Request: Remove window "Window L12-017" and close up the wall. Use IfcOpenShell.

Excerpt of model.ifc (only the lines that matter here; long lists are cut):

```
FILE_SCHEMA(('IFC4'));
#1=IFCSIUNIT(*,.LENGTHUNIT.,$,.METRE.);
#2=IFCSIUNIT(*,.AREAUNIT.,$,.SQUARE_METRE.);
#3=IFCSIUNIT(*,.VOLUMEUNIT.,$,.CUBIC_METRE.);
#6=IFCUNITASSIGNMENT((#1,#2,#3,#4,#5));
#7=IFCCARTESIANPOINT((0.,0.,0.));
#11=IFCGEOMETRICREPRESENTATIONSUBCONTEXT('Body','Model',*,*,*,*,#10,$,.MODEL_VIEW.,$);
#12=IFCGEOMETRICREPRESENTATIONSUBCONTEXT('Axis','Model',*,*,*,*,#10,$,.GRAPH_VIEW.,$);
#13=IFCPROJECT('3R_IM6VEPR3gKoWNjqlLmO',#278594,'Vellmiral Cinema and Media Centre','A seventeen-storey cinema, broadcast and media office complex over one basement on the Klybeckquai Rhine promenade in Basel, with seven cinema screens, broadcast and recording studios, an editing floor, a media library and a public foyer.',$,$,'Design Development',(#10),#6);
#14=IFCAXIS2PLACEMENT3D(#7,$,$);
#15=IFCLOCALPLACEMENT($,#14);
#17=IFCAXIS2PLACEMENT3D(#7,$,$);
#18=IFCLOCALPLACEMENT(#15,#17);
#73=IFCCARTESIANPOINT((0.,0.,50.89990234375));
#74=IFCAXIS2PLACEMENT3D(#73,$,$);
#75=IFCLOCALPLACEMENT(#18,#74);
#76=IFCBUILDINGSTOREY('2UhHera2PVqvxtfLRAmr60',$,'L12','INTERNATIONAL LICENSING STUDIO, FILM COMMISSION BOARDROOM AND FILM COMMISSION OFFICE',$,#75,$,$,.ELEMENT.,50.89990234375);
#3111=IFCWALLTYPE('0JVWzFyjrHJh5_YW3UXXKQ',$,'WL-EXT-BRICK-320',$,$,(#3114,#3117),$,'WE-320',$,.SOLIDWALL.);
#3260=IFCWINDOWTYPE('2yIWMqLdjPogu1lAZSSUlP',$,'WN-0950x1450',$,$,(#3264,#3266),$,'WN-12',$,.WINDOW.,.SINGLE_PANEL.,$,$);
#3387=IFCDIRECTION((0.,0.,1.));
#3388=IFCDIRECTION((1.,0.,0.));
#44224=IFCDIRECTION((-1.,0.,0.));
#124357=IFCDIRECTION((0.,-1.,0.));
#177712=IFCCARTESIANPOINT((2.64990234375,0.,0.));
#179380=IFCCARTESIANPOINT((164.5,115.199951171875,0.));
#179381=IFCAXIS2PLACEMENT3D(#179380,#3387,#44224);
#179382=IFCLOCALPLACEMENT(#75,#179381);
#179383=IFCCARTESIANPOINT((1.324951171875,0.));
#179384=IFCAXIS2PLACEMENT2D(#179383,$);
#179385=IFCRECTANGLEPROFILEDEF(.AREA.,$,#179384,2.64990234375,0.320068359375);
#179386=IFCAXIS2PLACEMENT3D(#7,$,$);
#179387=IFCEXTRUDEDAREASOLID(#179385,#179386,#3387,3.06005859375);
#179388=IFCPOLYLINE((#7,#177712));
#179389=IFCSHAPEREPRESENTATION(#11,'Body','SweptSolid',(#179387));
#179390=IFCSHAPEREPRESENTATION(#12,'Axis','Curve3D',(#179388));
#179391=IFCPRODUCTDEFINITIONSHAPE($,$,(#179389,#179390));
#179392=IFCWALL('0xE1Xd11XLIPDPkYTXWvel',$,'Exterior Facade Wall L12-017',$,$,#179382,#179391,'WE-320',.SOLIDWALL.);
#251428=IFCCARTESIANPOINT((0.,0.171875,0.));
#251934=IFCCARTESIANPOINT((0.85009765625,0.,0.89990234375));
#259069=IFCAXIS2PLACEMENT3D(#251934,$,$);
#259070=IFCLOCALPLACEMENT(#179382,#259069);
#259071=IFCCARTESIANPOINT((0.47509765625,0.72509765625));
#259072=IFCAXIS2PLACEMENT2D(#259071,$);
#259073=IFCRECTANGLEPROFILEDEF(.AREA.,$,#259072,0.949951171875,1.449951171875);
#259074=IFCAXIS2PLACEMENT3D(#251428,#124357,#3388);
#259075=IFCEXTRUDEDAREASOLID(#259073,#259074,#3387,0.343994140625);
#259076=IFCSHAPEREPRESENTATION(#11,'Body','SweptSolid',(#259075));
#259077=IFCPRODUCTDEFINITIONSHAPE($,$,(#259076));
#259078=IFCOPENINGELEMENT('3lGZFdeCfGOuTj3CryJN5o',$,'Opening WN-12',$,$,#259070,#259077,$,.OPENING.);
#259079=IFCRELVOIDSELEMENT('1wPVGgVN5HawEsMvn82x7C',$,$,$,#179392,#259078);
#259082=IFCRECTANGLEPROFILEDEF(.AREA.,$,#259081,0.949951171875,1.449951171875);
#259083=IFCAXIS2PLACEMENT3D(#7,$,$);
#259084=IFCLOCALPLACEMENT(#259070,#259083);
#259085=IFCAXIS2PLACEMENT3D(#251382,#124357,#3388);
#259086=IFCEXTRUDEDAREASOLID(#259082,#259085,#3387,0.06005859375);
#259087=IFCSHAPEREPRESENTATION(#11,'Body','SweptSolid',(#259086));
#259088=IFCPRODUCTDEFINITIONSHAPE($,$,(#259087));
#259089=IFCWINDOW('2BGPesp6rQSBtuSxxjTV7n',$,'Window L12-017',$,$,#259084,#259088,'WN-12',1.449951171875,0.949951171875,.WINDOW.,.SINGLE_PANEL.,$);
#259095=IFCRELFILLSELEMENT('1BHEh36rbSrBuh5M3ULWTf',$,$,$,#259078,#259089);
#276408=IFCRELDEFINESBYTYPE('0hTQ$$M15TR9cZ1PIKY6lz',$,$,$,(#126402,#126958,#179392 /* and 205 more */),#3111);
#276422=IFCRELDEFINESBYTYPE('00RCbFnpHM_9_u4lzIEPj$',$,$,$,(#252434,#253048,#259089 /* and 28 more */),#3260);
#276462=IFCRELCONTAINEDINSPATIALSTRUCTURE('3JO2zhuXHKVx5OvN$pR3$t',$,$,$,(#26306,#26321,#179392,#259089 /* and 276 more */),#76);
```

```python
import ifcopenshell
import ifcopenshell.api.feature
import ifcopenshell.api.root
import ifcopenshell.geom
import ifcopenshell.util.shape

model = ifcopenshell.open("model.ifc")
settings = ifcopenshell.geom.settings()


def volume(element):
    """Net volume in cubic metres, openings subtracted."""
    shape = ifcopenshell.geom.create_shape(settings, element)
    return ifcopenshell.util.shape.get_volume(shape.geometry)


window = model.by_id(259089)
opening = window.FillsVoids[0].RelatingOpeningElement
wall = opening.VoidsElements[0].RelatingBuildingElement
before = volume(wall)

ifcopenshell.api.root.remove_product(model, product=window)
ifcopenshell.api.feature.remove_feature(model, feature=opening)

after = volume(wall)

print(f"wall volume {before:.3f} -> {after:.3f} m3")

model.write("model_edited.ifc")
```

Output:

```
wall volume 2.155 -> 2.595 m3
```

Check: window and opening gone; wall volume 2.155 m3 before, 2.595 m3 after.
